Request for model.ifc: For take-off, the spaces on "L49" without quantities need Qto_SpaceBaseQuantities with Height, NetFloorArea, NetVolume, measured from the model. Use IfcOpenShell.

First a look at what the model holds.

```python
import ifcopenshell
import ifcopenshell.util.element
import ifcopenshell.util.unit

model = ifcopenshell.open("model.ifc")
print(model.schema)
for unit_type in ("LENGTHUNIT", "AREAUNIT", "VOLUMEUNIT"):
    print(unit_type, ifcopenshell.util.unit.calculate_unit_scale(model, unit_type))
storey = next(s for s in model.by_type("IfcBuildingStorey") if s.Name == "L49")
spaces = [e for e in ifcopenshell.util.element.get_decomposition(storey) if e.is_a("IfcSpace")]
for e in sorted(spaces, key=lambda e: e.id()):
    print(e.id(), e.is_a(), e.Name, list(ifcopenshell.util.element.get_psets(e, qtos_only=True)), sep=" | ")
```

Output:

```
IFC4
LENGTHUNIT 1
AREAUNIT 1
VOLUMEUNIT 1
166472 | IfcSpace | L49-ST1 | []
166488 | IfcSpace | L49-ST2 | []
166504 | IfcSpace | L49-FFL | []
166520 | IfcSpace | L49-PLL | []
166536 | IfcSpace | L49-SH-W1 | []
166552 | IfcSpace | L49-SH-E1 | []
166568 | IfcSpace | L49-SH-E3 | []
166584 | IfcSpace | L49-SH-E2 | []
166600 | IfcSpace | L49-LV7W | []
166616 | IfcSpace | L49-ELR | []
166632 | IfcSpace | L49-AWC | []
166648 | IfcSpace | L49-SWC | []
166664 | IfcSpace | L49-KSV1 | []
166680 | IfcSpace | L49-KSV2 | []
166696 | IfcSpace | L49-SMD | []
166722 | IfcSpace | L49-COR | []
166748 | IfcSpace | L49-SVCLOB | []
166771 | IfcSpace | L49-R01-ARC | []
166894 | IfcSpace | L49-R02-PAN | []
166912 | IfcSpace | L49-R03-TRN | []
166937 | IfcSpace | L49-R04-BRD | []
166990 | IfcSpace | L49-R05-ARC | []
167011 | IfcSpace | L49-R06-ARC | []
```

```python
import ifcopenshell
import ifcopenshell.api.pset
import ifcopenshell.geom
import ifcopenshell.util.element
import ifcopenshell.util.shape
import ifcopenshell.util.unit

model = ifcopenshell.open("model.ifc")
unit_scale = ifcopenshell.util.unit.calculate_unit_scale(model)
area_scale = ifcopenshell.util.unit.calculate_unit_scale(model, "AREAUNIT")
volume_scale = ifcopenshell.util.unit.calculate_unit_scale(model, "VOLUMEUNIT")
settings = ifcopenshell.geom.settings()

storey = next(s for s in model.by_type("IfcBuildingStorey") if s.Name == "L49")
spaces = [e for e in ifcopenshell.util.element.get_decomposition(storey) if e.is_a("IfcSpace")]

for e in sorted(spaces, key=lambda e: e.id()):
    if ifcopenshell.util.element.get_psets(e, qtos_only=True, should_inherit=False):
        continue
    # Geometry comes back in metres, in the element's own axes.
    shape = ifcopenshell.geom.create_shape(settings, e)
    values = {
        "Height": ifcopenshell.util.shape.get_z(shape.geometry) / unit_scale,
        "NetFloorArea": ifcopenshell.util.shape.get_footprint_area(shape.geometry) / area_scale,
        "NetVolume": ifcopenshell.util.shape.get_volume(shape.geometry) / volume_scale,
    }
    qto = ifcopenshell.api.pset.add_qto(model, product=e, name="Qto_SpaceBaseQuantities")
    ifcopenshell.api.pset.edit_qto(model, qto=qto, properties=values)
    print(e.id(), {k: round(v, 3) for k, v in values.items()})

model.write("model_edited.ifc")
```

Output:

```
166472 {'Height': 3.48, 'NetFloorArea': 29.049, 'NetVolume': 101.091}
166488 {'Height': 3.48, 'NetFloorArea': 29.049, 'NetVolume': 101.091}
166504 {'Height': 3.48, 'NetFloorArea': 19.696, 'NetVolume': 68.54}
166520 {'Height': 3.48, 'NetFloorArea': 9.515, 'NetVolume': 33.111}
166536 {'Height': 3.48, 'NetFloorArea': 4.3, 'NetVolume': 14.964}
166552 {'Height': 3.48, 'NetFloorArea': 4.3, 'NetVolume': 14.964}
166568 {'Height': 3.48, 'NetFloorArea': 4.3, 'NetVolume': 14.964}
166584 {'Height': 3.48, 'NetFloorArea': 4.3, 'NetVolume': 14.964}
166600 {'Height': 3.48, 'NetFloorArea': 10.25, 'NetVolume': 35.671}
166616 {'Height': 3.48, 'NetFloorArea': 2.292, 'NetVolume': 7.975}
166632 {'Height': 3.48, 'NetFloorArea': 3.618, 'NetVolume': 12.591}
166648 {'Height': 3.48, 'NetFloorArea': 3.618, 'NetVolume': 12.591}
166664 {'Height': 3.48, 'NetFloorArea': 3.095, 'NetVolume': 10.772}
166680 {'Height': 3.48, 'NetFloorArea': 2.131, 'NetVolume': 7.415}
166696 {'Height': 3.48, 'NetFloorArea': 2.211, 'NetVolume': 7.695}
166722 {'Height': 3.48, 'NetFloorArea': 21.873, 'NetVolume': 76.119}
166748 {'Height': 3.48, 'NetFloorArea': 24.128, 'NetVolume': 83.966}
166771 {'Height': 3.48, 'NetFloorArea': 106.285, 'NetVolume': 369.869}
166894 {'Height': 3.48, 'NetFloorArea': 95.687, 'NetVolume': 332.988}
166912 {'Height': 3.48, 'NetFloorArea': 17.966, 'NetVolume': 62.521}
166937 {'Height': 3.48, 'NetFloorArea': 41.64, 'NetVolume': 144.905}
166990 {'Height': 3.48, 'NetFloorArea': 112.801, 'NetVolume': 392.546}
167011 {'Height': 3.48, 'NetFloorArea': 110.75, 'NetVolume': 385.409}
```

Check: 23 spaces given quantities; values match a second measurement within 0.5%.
